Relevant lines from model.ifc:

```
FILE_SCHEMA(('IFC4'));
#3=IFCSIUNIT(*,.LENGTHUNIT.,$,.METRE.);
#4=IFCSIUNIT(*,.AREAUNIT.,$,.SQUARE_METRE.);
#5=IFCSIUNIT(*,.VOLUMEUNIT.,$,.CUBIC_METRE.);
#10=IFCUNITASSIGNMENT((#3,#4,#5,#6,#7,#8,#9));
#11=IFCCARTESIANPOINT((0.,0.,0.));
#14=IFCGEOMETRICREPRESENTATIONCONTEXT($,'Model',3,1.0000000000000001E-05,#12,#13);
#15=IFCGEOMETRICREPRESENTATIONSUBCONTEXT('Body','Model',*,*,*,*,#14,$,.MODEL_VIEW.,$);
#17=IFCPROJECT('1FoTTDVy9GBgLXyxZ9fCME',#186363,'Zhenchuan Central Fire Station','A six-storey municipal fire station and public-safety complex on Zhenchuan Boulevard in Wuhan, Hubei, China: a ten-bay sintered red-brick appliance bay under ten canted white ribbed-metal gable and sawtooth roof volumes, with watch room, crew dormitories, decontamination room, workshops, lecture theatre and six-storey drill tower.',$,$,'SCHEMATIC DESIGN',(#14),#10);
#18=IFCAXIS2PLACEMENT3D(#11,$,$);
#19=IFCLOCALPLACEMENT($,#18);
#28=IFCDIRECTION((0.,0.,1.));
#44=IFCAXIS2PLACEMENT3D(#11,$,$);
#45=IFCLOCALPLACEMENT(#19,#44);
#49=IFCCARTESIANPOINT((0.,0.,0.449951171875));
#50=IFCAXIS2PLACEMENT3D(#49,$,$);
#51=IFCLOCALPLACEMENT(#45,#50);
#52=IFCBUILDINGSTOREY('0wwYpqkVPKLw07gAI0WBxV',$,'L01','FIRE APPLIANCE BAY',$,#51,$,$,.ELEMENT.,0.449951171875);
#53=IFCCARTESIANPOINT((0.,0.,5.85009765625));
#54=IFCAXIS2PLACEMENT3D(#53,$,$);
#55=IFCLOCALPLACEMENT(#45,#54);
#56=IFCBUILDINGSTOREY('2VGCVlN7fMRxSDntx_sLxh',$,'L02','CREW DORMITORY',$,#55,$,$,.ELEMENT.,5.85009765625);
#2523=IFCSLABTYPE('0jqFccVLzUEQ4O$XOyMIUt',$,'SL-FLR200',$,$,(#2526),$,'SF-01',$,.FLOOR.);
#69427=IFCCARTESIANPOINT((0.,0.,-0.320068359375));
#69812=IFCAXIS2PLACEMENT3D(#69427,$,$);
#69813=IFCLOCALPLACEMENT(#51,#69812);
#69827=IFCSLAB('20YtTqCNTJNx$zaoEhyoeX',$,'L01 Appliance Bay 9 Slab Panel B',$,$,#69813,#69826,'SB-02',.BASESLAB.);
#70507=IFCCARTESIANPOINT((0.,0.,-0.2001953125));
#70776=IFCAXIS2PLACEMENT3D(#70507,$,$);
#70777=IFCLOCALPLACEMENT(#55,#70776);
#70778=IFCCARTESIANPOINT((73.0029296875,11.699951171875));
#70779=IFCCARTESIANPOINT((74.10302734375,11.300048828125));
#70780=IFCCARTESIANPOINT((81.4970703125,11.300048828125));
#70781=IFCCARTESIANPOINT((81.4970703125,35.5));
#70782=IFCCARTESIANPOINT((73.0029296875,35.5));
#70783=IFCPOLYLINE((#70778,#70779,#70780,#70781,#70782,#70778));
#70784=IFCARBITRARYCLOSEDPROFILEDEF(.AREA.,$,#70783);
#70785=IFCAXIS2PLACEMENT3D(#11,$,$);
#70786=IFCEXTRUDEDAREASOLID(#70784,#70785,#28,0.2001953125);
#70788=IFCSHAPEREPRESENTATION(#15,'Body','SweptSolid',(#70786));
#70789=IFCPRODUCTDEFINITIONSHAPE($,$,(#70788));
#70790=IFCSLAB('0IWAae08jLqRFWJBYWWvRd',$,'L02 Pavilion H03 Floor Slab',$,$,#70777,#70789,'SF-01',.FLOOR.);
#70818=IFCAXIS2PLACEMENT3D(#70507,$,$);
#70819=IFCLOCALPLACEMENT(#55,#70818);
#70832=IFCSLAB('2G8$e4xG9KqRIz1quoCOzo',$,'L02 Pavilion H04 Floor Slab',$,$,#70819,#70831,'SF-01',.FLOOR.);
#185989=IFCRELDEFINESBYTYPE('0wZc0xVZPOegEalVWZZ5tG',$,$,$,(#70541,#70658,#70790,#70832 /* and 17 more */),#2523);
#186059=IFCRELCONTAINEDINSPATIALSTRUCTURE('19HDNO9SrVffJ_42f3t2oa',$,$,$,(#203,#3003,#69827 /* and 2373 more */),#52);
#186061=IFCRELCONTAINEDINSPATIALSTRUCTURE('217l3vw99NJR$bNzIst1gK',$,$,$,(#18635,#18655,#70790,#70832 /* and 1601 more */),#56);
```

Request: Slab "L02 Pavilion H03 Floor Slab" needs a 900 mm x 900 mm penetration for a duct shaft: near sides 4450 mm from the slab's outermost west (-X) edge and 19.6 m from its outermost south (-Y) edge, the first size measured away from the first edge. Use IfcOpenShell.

```python
import numpy as np
import ifcopenshell
import ifcopenshell.api.feature
import ifcopenshell.api.geometry
import ifcopenshell.api.root
import ifcopenshell.geom
import ifcopenshell.util.placement
import ifcopenshell.util.representation
import ifcopenshell.util.shape
import ifcopenshell.util.unit

model = ifcopenshell.open("model.ifc")
unit_scale = ifcopenshell.util.unit.calculate_unit_scale(model)
settings = ifcopenshell.geom.settings()


def volume(element):
    """Net volume in cubic metres, openings subtracted."""
    shape = ifcopenshell.geom.create_shape(settings, element)
    return ifcopenshell.util.shape.get_volume(shape.geometry)


slab = model.by_id(70790)
before = volume(slab)

# Extent in the slab's own axes, in metres. The edges named are its -X and -Y sides.
slab_shape = ifcopenshell.geom.create_shape(settings, slab)
vertices = ifcopenshell.util.shape.get_vertices(slab_shape.geometry)
x_min, y_min, bottom = vertices.min(axis=0)
top = vertices[:, 2].max()

opening = ifcopenshell.api.root.create_entity(model, ifc_class="IfcOpeningElement", name="Duct shaft opening", predefined_type="OPENING")
context = ifcopenshell.util.representation.get_context(model, "Model", "Body", "MODEL_VIEW")
width, depth = 0.9, 0.9
outline = [(0.0, 0.0), (width, 0.0), (width, depth), (0.0, depth), (0.0, 0.0)]
# Overshoot both faces by 50 mm so the cut is clean.
shape = ifcopenshell.api.geometry.add_slab_representation(
    model, context=context, depth=top - bottom + 0.1, polyline=outline
)
ifcopenshell.api.geometry.assign_representation(model, product=opening, representation=shape)

matrix = ifcopenshell.util.placement.get_local_placement(slab.ObjectPlacement)
matrix[:, 3] = matrix @ np.append(np.array([x_min + 4.45, y_min + 19.6, bottom - 0.05]) / unit_scale, 1.0)
ifcopenshell.api.geometry.edit_object_placement(model, product=opening, matrix=matrix, is_si=False)
ifcopenshell.api.feature.add_feature(model, feature=opening, element=slab)

after = volume(slab)

print(f"slab volume {before:.3f} -> {after:.3f} m3")

model.write("model_edited.ifc")
```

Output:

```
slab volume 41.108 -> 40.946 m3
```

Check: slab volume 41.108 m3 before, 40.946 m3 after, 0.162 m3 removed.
